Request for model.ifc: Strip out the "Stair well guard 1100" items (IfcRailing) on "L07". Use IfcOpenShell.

First a look at what the model holds.

```python
import ifcopenshell
import ifcopenshell.util.element

model = ifcopenshell.open("model.ifc")
print(model.schema)
storey = next(s for s in model.by_type("IfcBuildingStorey") if s.Name == "L07")
railings = [e for e in ifcopenshell.util.element.get_decomposition(storey) if e.is_a("IfcRailing")]
seen = {}
for e in railings:
    element_type = ifcopenshell.util.element.get_type(e)
    name = element_type.Name if element_type not in (None, e) else None
    seen[name] = seen.get(name, 0) + 1
for name, count in sorted(seen.items(), key=str):
    print(count, "x", name)
```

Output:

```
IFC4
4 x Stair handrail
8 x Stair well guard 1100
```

```python
import ifcopenshell
import ifcopenshell.api.root
import ifcopenshell.util.element

model = ifcopenshell.open("model.ifc")

storey = next(s for s in model.by_type("IfcBuildingStorey") if s.Name == "L07")
railings = [e for e in ifcopenshell.util.element.get_decomposition(storey) if e.is_a("IfcRailing")]
targets = [e for e in railings if (t := ifcopenshell.util.element.get_type(e)) not in (None, e) and t.Name == "Stair well guard 1100"]

for e in targets:
    ifcopenshell.api.root.remove_product(model, product=e)
print(len(targets), "removed")

model.write("model_v2.ifc")
```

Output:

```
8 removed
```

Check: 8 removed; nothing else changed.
